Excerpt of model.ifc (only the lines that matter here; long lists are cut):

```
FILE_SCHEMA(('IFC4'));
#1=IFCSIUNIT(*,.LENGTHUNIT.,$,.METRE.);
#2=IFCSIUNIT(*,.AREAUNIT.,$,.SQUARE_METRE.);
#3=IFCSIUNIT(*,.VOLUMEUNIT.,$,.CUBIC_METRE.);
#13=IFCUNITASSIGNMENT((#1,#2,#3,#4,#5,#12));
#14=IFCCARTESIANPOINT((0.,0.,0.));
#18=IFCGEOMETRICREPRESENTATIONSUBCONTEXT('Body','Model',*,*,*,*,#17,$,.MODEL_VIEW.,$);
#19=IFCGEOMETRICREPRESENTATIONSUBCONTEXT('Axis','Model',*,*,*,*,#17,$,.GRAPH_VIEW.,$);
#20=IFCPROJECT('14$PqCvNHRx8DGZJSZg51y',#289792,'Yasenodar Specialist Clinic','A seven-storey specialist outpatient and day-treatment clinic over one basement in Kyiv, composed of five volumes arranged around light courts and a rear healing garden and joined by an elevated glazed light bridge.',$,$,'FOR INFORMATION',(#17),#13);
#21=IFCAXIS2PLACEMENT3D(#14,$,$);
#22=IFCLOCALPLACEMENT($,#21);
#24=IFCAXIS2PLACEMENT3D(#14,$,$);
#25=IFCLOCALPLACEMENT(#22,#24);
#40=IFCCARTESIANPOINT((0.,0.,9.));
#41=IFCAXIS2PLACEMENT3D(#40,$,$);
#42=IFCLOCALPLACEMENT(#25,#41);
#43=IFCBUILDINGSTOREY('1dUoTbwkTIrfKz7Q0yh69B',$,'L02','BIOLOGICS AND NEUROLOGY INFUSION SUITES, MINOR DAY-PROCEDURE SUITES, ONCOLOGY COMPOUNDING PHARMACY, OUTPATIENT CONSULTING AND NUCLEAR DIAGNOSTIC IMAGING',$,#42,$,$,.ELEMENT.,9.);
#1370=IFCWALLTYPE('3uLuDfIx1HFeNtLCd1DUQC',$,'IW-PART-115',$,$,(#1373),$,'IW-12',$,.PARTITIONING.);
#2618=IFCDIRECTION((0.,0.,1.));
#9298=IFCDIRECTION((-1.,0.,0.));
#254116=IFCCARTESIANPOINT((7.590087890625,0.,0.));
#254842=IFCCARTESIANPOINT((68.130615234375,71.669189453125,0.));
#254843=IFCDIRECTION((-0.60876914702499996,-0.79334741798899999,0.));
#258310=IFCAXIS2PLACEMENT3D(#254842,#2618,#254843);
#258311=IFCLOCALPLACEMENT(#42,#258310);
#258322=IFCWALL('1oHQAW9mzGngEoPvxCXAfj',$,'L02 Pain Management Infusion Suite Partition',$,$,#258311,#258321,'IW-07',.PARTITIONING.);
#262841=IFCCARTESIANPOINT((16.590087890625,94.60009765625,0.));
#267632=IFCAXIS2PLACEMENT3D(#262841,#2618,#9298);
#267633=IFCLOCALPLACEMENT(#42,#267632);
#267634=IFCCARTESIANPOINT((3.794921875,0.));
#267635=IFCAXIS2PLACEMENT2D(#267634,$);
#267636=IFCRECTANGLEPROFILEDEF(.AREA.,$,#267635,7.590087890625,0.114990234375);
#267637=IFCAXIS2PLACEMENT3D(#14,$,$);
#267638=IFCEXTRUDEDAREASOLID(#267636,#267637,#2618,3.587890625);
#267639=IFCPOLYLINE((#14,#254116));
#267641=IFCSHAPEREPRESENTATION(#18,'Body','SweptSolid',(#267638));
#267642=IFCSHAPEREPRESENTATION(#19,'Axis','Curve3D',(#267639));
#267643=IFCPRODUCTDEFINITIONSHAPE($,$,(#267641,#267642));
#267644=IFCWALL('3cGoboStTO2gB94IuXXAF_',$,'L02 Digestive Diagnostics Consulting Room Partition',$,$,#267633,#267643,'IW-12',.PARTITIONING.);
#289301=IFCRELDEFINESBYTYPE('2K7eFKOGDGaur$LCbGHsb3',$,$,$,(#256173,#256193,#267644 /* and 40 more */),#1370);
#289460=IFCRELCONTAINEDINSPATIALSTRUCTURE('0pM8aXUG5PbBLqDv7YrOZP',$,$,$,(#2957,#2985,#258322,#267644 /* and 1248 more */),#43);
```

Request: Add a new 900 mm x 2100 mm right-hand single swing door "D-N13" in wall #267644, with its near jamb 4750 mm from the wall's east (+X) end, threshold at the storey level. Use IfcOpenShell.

```python
import numpy as np
import ifcopenshell
import ifcopenshell.api.feature
import ifcopenshell.api.geometry
import ifcopenshell.api.root
import ifcopenshell.api.spatial
import ifcopenshell.geom
import ifcopenshell.util.element
import ifcopenshell.util.placement
import ifcopenshell.util.representation
import ifcopenshell.util.shape
import ifcopenshell.util.unit

model = ifcopenshell.open("model.ifc")
unit_scale = ifcopenshell.util.unit.calculate_unit_scale(model)
settings = ifcopenshell.geom.settings()


def volume(element):
    """Net volume in cubic metres, openings subtracted."""
    shape = ifcopenshell.geom.create_shape(settings, element)
    return ifcopenshell.util.shape.get_volume(shape.geometry)


wall = model.by_guid("3cGoboStTO2gB94IuXXAF_")
storey = ifcopenshell.util.element.get_container(wall, ifc_class="IfcBuildingStorey")
context = ifcopenshell.util.representation.get_context(model, "Model", "Body", "MODEL_VIEW")
before = volume(wall)

width, height, from_end, sill = 0.9, 2.1, 4.75, 0.0  # metres

# The wall runs along its own X axis, and the end named is its -X end.
wall_shape = ifcopenshell.geom.create_shape(settings, wall)
x, y, z = ifcopenshell.util.shape.get_vertices(wall_shape.geometry).T
start = x.min() + from_end
face, thickness = float(y.min()), float(y.max() - y.min())
wall_matrix = ifcopenshell.util.placement.get_local_placement(wall.ObjectPlacement)
level = ifcopenshell.util.placement.get_local_placement(storey.ObjectPlacement)[2, 3]


def in_wall(x, y):
    """Placement at x, y metres in the wall's axes, at sill height."""
    matrix = wall_matrix.copy()
    matrix[:, 3] = wall_matrix @ np.array([x / unit_scale, y / unit_scale, 0.0, 1.0])
    matrix[2, 3] = level + sill / unit_scale
    return matrix


# Opening: a box that overshoots both wall faces by 50 mm.
opening = ifcopenshell.api.root.create_entity(model, ifc_class="IfcOpeningElement", predefined_type="OPENING")
box = ifcopenshell.api.geometry.add_wall_representation(
    model, context=context, length=width, height=height, thickness=thickness + 0.1
)
ifcopenshell.api.geometry.assign_representation(model, product=opening, representation=box)
ifcopenshell.api.geometry.edit_object_placement(model, product=opening, matrix=in_wall(start, face - 0.05), is_si=False)
ifcopenshell.api.feature.add_feature(model, feature=opening, element=wall)

door = ifcopenshell.api.root.create_entity(model, ifc_class="IfcDoor", name="D-N13", predefined_type="DOOR")
door.OverallWidth, door.OverallHeight = width / unit_scale, height / unit_scale
door.OperationType = "SINGLE_SWING_RIGHT"
body = ifcopenshell.api.geometry.add_door_representation(
    model,
    context=context,
    overall_width=door.OverallWidth,
    overall_height=door.OverallHeight,
    operation_type="SINGLE_SWING_RIGHT",
    lining_properties={"LiningDepth": thickness / unit_scale, "ThresholdDepth": thickness / unit_scale},
)
ifcopenshell.api.geometry.assign_representation(model, product=door, representation=body)
ifcopenshell.api.spatial.assign_container(model, products=[door], relating_structure=storey)
ifcopenshell.api.feature.add_filling(model, opening=opening, element=door)

# The lining spans the wall, so the door starts at the wall face.
ifcopenshell.api.geometry.edit_object_placement(model, product=door, matrix=in_wall(start, face), is_si=False)

after = volume(wall)

print(f"wall volume {before:.3f} -> {after:.3f} m3")

model.write("model_updated.ifc")
```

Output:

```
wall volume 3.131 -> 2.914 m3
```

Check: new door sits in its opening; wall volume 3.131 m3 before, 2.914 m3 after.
